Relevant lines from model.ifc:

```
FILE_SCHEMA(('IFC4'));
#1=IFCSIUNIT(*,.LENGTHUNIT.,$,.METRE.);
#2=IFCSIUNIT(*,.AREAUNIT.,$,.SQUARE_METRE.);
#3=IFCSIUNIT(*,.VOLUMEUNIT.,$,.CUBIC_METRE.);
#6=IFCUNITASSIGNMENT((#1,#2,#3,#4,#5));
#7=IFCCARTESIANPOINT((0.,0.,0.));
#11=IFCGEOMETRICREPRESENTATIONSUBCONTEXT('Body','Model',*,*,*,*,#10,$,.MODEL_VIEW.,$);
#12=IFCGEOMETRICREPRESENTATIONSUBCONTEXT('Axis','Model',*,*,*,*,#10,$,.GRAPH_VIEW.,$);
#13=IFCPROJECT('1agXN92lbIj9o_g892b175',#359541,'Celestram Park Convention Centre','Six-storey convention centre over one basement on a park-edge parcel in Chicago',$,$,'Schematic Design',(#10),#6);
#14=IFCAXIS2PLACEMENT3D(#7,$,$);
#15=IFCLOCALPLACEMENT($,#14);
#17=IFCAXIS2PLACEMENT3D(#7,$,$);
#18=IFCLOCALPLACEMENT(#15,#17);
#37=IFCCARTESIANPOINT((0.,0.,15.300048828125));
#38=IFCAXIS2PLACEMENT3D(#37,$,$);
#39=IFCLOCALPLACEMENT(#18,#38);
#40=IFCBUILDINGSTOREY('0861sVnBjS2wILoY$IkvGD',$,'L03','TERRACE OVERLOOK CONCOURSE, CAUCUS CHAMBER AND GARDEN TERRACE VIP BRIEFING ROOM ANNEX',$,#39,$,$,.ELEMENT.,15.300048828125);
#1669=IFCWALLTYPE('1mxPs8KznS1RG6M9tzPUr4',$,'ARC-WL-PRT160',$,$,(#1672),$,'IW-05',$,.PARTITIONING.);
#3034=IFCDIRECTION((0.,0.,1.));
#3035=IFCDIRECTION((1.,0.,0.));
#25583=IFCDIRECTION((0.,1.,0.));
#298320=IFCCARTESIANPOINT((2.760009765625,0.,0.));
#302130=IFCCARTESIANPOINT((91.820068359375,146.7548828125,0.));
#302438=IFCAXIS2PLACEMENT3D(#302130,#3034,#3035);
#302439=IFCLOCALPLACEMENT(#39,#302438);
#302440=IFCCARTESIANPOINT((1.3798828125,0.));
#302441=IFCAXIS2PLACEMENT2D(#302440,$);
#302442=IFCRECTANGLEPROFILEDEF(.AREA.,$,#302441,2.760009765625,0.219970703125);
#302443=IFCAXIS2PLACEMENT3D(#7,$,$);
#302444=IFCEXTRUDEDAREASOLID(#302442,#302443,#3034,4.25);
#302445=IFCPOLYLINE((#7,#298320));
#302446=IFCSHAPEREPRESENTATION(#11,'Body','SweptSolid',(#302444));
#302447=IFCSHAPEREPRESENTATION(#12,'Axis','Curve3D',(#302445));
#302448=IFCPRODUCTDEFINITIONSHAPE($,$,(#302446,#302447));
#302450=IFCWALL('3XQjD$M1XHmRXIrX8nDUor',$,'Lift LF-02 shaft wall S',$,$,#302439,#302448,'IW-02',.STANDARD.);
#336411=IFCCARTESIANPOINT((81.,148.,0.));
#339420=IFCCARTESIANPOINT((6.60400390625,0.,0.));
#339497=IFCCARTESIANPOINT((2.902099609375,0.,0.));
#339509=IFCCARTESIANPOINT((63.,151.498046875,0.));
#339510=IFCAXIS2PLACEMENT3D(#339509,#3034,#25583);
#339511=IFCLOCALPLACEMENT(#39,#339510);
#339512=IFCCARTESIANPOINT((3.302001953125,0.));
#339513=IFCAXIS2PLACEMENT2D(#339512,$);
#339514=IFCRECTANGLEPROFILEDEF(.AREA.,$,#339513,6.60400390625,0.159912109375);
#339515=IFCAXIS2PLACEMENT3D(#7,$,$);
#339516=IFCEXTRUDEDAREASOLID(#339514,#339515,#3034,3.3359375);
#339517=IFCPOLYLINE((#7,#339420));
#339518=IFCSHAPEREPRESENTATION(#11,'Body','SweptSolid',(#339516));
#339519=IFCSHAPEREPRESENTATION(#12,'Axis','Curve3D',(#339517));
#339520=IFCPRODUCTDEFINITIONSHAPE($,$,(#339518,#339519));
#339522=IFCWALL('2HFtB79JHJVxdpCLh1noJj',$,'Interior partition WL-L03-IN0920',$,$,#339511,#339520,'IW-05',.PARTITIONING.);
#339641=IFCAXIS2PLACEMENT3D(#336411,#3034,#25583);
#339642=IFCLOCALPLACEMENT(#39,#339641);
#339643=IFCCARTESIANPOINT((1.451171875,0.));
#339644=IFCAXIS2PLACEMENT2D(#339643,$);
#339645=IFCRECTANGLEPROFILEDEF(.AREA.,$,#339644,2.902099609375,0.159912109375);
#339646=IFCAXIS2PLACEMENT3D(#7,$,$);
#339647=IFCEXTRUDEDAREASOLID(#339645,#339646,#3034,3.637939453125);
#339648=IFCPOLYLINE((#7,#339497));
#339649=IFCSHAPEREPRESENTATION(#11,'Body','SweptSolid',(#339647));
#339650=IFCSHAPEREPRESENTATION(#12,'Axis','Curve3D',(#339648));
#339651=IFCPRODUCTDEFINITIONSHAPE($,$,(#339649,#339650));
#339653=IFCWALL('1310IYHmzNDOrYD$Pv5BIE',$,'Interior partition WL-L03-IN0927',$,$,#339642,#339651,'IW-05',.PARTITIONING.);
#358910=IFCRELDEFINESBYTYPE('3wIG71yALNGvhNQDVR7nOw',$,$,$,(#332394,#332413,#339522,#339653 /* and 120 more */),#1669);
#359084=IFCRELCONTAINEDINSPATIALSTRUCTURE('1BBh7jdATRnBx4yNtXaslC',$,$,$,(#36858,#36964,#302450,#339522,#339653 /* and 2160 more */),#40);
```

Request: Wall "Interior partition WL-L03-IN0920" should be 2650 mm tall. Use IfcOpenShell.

```python
import ifcopenshell
import ifcopenshell.geom
import ifcopenshell.util.representation
import ifcopenshell.util.shape
import ifcopenshell.util.unit

model = ifcopenshell.open("model.ifc")
unit_scale = ifcopenshell.util.unit.calculate_unit_scale(model)
settings = ifcopenshell.geom.settings()


def volume(element):
    """Net volume in cubic metres, openings subtracted."""
    shape = ifcopenshell.geom.create_shape(settings, element)
    return ifcopenshell.util.shape.get_volume(shape.geometry)


wall = model.by_guid("2HFtB79JHJVxdpCLh1noJj")
before = volume(wall)

body = ifcopenshell.util.representation.get_representation(wall, "Model", "Body")
solid = body.Items[0]
old_height = solid.Depth
solid.Depth = 2.65 / unit_scale
after = volume(wall)

print(f"height {old_height:g} -> {solid.Depth:g}, volume {before:.3f} -> {after:.3f} m3")

model.write("model_updated.ifc")
```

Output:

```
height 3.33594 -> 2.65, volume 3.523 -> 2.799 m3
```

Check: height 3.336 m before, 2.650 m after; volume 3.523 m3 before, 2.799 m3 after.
